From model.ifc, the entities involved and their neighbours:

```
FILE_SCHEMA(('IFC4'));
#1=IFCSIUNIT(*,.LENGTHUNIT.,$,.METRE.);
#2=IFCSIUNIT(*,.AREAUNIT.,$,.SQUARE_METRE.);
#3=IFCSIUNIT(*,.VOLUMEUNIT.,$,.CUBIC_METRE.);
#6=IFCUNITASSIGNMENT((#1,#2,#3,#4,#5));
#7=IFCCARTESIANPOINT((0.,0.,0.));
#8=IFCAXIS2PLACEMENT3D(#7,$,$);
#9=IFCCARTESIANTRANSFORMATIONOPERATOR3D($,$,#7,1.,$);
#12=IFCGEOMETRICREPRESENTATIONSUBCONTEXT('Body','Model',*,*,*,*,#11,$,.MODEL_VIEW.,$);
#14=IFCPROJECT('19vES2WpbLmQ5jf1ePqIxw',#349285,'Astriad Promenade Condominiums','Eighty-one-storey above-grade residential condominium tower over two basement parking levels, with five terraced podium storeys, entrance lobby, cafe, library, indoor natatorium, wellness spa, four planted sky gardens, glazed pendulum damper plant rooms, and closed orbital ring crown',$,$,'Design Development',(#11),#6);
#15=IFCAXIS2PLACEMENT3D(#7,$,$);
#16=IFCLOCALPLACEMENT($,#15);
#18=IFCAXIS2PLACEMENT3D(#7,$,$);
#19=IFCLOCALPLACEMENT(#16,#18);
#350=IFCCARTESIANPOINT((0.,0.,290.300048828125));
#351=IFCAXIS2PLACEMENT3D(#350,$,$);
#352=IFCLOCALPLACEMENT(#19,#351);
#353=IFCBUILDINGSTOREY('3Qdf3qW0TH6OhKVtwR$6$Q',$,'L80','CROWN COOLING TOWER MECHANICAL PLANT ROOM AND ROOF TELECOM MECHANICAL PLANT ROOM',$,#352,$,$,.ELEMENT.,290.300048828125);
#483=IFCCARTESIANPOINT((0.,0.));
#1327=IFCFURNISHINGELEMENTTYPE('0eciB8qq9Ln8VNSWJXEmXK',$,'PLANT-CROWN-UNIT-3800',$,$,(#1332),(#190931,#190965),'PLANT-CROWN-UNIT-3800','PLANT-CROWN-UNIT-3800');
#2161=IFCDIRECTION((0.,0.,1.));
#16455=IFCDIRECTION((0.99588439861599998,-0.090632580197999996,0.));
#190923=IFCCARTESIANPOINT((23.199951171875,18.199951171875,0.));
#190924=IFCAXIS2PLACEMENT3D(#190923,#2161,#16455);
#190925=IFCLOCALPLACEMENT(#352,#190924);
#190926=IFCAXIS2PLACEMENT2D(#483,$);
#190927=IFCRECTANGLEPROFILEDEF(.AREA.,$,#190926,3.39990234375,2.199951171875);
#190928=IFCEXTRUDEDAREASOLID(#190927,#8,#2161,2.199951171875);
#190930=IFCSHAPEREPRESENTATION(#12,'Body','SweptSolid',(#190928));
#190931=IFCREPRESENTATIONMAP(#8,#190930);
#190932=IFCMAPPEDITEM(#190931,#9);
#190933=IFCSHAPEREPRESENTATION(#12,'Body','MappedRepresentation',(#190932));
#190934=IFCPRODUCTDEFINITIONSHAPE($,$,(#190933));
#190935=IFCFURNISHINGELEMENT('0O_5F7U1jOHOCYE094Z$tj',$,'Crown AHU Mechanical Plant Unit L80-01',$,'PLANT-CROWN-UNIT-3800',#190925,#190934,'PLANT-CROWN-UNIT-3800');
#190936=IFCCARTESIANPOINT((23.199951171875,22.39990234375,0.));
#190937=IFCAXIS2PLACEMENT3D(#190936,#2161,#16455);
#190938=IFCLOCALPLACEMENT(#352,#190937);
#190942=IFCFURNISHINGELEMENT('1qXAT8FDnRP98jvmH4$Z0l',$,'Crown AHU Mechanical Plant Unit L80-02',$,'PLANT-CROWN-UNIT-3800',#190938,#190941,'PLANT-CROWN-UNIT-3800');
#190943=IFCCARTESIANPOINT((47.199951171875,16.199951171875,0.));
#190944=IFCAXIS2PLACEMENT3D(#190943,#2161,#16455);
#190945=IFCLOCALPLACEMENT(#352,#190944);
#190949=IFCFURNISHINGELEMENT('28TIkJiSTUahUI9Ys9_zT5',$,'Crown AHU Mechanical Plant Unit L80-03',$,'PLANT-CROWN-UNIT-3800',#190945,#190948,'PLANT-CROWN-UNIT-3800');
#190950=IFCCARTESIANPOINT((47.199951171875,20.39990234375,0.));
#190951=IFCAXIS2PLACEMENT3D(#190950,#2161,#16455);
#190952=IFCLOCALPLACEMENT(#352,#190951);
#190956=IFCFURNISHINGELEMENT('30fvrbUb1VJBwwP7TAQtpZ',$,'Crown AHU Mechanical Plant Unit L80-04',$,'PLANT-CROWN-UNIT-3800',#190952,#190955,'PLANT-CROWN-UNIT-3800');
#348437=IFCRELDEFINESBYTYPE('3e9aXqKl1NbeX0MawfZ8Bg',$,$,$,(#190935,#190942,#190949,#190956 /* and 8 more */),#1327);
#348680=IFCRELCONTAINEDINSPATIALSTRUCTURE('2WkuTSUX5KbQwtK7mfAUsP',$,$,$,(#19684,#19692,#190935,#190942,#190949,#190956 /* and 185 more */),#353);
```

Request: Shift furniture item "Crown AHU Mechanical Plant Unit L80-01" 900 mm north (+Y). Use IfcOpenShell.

```python
import ifcopenshell
import ifcopenshell.api.geometry
import ifcopenshell.util.placement

model = ifcopenshell.open("model.ifc")

item = model.by_guid("0O_5F7U1jOHOCYE094Z$tj")
matrix = ifcopenshell.util.placement.get_local_placement(item.ObjectPlacement)
matrix[1, 3] += 0.9
ifcopenshell.api.geometry.edit_object_placement(model, product=item, matrix=matrix, is_si=False)

print(ifcopenshell.util.placement.get_local_placement(item.ObjectPlacement).round(3) + 0.0)

model.write("model_edited.ifc")
```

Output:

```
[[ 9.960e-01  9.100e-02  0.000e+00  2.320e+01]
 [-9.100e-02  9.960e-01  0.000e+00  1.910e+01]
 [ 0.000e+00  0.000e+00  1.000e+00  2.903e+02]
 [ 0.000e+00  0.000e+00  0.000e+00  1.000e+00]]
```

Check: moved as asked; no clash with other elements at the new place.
